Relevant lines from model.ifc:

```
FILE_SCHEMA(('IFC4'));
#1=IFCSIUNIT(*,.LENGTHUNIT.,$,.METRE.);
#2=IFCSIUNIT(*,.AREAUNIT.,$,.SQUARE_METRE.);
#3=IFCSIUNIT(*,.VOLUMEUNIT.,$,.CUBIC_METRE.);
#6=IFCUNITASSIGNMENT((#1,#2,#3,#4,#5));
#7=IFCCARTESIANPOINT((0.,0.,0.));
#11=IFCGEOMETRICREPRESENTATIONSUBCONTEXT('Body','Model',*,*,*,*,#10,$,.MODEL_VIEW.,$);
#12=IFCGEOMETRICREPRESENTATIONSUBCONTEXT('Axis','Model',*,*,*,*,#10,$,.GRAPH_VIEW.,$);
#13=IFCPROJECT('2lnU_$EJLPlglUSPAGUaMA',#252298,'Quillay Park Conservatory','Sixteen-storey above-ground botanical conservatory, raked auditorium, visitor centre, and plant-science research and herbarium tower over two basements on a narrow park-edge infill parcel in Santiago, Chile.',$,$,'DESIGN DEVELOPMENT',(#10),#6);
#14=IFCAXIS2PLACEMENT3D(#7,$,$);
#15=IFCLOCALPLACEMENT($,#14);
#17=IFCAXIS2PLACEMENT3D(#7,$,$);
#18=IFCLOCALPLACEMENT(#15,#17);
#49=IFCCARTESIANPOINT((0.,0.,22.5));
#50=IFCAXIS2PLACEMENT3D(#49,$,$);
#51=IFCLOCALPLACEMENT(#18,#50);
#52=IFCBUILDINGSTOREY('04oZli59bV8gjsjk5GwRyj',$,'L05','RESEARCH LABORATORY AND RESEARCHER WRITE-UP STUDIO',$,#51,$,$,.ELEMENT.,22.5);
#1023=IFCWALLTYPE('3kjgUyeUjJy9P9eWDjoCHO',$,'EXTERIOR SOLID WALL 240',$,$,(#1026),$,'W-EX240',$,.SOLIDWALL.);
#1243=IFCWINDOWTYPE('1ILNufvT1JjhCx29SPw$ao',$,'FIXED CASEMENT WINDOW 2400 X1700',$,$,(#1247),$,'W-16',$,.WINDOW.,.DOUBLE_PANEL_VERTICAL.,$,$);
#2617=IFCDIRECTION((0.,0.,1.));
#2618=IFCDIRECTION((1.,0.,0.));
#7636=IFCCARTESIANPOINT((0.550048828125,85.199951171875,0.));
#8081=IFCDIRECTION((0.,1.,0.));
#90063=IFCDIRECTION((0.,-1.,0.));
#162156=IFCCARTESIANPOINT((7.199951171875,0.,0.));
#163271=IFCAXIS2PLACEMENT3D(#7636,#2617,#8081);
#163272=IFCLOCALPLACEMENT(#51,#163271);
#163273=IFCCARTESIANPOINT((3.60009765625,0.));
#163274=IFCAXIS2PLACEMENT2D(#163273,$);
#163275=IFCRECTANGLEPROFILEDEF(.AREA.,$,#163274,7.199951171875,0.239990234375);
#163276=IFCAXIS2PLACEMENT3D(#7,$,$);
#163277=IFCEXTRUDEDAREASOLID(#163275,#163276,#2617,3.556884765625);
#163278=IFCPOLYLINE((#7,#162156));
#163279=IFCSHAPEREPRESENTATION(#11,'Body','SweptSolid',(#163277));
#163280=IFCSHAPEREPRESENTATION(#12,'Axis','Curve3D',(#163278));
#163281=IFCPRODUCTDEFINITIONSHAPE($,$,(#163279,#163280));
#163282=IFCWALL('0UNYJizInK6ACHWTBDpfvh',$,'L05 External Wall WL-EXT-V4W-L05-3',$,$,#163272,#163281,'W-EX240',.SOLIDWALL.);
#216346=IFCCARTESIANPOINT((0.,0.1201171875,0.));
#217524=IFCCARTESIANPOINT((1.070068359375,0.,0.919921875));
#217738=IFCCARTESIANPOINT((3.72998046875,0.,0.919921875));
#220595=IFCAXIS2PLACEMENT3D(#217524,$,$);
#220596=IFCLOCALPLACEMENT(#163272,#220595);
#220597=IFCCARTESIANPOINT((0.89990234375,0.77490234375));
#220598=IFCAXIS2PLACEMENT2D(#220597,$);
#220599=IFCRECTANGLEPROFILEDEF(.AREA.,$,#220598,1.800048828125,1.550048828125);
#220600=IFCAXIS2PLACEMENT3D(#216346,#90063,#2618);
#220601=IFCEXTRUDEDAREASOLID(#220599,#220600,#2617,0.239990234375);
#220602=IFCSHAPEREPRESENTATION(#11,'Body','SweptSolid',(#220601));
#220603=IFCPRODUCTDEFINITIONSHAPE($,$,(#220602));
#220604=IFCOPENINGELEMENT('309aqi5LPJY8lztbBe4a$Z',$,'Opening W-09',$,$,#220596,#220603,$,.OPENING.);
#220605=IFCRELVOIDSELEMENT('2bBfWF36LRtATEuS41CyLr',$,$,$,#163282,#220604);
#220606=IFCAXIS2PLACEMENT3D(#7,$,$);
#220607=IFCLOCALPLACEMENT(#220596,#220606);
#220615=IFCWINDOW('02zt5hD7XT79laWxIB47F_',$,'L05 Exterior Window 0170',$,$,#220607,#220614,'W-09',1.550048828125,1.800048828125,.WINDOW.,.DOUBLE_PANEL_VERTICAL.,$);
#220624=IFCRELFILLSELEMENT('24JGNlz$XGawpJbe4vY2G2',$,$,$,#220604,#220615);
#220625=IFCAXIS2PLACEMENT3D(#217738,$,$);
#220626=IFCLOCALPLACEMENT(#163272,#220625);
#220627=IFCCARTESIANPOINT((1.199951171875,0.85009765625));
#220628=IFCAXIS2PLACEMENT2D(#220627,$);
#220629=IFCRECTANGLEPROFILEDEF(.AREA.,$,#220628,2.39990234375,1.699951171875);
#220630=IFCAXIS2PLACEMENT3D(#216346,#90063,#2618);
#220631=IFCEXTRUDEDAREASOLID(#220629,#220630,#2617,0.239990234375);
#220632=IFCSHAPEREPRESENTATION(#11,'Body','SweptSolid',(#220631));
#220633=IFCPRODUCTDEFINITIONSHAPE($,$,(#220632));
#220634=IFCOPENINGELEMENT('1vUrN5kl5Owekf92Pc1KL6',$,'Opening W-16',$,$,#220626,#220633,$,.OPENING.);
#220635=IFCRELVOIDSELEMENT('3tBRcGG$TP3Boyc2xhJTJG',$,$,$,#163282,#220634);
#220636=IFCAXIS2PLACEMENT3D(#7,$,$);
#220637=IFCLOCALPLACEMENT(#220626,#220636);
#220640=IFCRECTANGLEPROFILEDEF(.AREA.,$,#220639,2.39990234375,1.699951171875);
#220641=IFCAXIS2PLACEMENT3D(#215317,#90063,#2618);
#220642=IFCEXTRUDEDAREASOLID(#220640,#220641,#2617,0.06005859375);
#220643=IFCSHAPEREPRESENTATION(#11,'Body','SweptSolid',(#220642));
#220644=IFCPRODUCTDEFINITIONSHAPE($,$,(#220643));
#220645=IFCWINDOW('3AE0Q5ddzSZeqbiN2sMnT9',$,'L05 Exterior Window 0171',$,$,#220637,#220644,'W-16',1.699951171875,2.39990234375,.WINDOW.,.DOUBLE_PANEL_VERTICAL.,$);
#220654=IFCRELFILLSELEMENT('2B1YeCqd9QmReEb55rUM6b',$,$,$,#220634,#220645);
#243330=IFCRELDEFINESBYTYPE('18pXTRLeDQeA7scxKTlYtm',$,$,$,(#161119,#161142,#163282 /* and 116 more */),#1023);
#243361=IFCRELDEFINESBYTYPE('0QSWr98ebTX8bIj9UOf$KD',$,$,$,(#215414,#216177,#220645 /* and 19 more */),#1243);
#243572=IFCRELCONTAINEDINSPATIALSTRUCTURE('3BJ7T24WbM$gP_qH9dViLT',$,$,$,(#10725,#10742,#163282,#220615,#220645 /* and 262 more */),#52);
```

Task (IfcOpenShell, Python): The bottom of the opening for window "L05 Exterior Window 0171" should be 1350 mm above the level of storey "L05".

```python
import numpy as np
import ifcopenshell
import ifcopenshell.api.geometry
import ifcopenshell.geom
import ifcopenshell.util.element
import ifcopenshell.util.placement
import ifcopenshell.util.shape
import ifcopenshell.util.unit

model = ifcopenshell.open("model.ifc")
unit_scale = ifcopenshell.util.unit.calculate_unit_scale(model)

window = model.by_id(220645)
opening = window.FillsVoids[0].RelatingOpeningElement
storey = ifcopenshell.util.element.get_container(window, ifc_class="IfcBuildingStorey")
level = ifcopenshell.util.placement.get_local_placement(storey.ObjectPlacement)[2, 3]

# The opening's origin need not be at the sill, so measure its lowest point.
shape = ifcopenshell.geom.create_shape(ifcopenshell.geom.settings(), opening)
bottom = ifcopenshell.util.shape.get_shape_bottom_elevation(shape, shape.geometry) / unit_scale
dz = level + 1.35 / unit_scale - bottom

shift = np.array([0.0, 0.0, dz])
# The window is placed relative to its opening, so it follows when the opening moves.
matrix = ifcopenshell.util.placement.get_local_placement(opening.ObjectPlacement)
matrix[:3, 3] += shift
ifcopenshell.api.geometry.edit_object_placement(
    model, product=opening, matrix=matrix, is_si=False, should_transform_children=True
)

print(f"moved by {dz * unit_scale:+.3f} m")

model.write("model-out.ifc")
```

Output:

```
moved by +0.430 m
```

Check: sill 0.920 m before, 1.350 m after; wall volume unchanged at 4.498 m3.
